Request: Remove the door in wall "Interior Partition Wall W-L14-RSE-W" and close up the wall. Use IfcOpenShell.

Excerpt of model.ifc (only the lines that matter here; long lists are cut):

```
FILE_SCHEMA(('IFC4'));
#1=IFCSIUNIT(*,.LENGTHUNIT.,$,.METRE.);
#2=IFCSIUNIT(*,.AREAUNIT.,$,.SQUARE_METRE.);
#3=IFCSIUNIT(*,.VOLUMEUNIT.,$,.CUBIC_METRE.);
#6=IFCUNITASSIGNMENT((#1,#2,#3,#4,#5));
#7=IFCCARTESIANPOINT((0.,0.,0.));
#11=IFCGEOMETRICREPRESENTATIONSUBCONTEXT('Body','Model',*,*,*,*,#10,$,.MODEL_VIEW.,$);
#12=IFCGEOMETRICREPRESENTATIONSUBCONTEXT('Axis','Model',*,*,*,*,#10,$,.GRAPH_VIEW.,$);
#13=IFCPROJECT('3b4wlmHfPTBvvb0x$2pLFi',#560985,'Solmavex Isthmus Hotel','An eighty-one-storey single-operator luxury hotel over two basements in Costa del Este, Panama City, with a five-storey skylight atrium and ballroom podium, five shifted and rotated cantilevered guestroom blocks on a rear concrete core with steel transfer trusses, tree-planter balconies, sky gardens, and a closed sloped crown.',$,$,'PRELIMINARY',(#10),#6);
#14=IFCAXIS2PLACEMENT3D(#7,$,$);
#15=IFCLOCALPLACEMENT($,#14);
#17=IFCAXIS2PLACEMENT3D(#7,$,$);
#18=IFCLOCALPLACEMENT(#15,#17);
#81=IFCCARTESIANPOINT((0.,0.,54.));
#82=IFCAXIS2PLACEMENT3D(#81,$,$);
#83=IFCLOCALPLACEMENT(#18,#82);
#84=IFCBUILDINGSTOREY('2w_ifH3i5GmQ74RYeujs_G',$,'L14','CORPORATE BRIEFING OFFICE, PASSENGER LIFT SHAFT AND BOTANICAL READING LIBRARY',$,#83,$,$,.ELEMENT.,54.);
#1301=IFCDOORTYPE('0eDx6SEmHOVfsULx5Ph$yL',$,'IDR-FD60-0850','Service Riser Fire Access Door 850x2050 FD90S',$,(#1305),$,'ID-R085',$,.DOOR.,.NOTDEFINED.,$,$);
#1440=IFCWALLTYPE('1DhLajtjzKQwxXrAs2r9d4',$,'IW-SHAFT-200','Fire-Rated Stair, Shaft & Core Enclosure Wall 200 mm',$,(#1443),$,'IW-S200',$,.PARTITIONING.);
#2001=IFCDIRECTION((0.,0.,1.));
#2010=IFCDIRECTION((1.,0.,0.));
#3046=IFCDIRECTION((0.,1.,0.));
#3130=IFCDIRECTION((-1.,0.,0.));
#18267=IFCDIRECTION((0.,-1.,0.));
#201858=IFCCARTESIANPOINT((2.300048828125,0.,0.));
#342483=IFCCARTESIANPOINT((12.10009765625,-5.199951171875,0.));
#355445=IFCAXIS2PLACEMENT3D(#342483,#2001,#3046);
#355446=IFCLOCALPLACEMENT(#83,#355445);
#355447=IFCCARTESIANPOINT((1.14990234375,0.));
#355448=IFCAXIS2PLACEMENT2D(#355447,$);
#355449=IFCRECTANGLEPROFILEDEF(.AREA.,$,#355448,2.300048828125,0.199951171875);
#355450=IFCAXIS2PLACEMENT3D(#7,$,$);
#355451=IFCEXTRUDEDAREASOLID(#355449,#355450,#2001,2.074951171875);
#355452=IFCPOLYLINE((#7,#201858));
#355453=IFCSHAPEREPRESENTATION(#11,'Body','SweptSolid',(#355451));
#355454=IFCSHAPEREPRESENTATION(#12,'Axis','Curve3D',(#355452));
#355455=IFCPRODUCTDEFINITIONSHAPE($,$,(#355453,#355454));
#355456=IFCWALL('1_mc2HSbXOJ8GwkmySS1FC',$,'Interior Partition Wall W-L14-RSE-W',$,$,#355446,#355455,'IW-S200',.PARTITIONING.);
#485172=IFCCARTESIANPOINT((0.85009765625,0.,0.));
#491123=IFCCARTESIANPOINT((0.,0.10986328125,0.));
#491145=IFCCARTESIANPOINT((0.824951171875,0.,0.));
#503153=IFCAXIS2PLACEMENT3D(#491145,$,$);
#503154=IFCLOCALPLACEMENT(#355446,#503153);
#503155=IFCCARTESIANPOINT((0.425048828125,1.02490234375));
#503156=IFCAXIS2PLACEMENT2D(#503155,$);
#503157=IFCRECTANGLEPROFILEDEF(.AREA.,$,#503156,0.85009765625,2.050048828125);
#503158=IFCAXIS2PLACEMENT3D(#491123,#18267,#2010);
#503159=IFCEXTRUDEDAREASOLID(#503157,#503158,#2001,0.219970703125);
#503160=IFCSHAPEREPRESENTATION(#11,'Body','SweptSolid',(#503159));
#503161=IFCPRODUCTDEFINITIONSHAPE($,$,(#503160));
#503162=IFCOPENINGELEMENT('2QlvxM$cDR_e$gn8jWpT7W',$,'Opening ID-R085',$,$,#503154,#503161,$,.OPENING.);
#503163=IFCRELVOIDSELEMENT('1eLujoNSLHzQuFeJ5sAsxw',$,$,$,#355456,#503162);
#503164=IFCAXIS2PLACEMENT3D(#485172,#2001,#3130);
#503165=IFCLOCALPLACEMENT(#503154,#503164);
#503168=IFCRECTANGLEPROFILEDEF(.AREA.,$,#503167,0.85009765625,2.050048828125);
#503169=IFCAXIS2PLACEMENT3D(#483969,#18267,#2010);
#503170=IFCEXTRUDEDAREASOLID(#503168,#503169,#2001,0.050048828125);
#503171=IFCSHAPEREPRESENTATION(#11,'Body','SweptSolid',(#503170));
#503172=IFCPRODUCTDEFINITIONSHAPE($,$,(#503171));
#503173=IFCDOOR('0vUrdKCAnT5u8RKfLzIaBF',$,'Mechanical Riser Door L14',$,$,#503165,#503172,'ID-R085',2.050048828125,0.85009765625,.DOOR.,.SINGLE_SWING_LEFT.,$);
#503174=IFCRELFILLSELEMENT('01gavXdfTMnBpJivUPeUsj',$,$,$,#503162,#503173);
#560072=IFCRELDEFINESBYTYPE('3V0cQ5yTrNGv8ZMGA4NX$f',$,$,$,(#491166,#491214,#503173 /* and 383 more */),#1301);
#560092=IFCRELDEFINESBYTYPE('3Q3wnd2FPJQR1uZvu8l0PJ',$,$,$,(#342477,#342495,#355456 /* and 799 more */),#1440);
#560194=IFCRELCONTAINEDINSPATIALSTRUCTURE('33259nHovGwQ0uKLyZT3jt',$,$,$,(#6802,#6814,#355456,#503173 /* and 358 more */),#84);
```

```python
import ifcopenshell
import ifcopenshell.api.feature
import ifcopenshell.api.root
import ifcopenshell.geom
import ifcopenshell.util.shape

model = ifcopenshell.open("model.ifc")
settings = ifcopenshell.geom.settings()


def volume(element):
    """Net volume in cubic metres, openings subtracted."""
    shape = ifcopenshell.geom.create_shape(settings, element)
    return ifcopenshell.util.shape.get_volume(shape.geometry)


door = model.by_guid("0vUrdKCAnT5u8RKfLzIaBF")
opening = door.FillsVoids[0].RelatingOpeningElement
wall = opening.VoidsElements[0].RelatingBuildingElement
before = volume(wall)

ifcopenshell.api.root.remove_product(model, product=door)
ifcopenshell.api.feature.remove_feature(model, feature=opening)

after = volume(wall)

print(f"wall volume {before:.3f} -> {after:.3f} m3")

model.write("model_edited.ifc")
```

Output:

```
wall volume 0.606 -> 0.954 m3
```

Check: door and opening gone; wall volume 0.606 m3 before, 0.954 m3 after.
